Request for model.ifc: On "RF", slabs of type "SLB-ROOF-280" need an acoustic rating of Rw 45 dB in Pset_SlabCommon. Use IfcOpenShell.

First a look at what the model holds.

```python
import ifcopenshell
import ifcopenshell.util.element

model = ifcopenshell.open("model.ifc")
print(model.schema)
storey = next(s for s in model.by_type("IfcBuildingStorey") if s.Name == "RF")
slabs = [e for e in ifcopenshell.util.element.get_decomposition(storey) if e.is_a("IfcSlab")]
seen = {}
for e in slabs:
    element_type = ifcopenshell.util.element.get_type(e)
    key = (element_type.Name if element_type != e and element_type else None, ifcopenshell.util.element.get_pset(e, "Pset_SlabCommon", "AcousticRating"))
    seen[key] = seen.get(key, 0) + 1
for (name, value), count in sorted(seen.items(), key=str):
    print(count, "x", name, "|", value)
```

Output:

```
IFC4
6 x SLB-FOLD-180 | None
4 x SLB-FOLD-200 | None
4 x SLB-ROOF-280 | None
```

```python
import ifcopenshell
import ifcopenshell.api.pset
import ifcopenshell.util.element

model = ifcopenshell.open("model.ifc")

storey = next(s for s in model.by_type("IfcBuildingStorey") if s.Name == "RF")
slabs = [e for e in ifcopenshell.util.element.get_decomposition(storey) if e.is_a("IfcSlab")]

count = 0
for e in slabs:
    element_type = ifcopenshell.util.element.get_type(e)
    if element_type in (None, e) or element_type.Name != "SLB-ROOF-280":
        continue
    # add_pset returns the element's existing set when there is one.
    pset = ifcopenshell.api.pset.add_pset(model, product=e, name="Pset_SlabCommon")
    ifcopenshell.api.pset.edit_pset(model, pset=pset, properties={"AcousticRating": "Rw 45 dB"})
    count += 1

print(count, "slabs updated")

model.write("model_updated.ifc")
```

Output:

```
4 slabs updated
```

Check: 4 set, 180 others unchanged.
